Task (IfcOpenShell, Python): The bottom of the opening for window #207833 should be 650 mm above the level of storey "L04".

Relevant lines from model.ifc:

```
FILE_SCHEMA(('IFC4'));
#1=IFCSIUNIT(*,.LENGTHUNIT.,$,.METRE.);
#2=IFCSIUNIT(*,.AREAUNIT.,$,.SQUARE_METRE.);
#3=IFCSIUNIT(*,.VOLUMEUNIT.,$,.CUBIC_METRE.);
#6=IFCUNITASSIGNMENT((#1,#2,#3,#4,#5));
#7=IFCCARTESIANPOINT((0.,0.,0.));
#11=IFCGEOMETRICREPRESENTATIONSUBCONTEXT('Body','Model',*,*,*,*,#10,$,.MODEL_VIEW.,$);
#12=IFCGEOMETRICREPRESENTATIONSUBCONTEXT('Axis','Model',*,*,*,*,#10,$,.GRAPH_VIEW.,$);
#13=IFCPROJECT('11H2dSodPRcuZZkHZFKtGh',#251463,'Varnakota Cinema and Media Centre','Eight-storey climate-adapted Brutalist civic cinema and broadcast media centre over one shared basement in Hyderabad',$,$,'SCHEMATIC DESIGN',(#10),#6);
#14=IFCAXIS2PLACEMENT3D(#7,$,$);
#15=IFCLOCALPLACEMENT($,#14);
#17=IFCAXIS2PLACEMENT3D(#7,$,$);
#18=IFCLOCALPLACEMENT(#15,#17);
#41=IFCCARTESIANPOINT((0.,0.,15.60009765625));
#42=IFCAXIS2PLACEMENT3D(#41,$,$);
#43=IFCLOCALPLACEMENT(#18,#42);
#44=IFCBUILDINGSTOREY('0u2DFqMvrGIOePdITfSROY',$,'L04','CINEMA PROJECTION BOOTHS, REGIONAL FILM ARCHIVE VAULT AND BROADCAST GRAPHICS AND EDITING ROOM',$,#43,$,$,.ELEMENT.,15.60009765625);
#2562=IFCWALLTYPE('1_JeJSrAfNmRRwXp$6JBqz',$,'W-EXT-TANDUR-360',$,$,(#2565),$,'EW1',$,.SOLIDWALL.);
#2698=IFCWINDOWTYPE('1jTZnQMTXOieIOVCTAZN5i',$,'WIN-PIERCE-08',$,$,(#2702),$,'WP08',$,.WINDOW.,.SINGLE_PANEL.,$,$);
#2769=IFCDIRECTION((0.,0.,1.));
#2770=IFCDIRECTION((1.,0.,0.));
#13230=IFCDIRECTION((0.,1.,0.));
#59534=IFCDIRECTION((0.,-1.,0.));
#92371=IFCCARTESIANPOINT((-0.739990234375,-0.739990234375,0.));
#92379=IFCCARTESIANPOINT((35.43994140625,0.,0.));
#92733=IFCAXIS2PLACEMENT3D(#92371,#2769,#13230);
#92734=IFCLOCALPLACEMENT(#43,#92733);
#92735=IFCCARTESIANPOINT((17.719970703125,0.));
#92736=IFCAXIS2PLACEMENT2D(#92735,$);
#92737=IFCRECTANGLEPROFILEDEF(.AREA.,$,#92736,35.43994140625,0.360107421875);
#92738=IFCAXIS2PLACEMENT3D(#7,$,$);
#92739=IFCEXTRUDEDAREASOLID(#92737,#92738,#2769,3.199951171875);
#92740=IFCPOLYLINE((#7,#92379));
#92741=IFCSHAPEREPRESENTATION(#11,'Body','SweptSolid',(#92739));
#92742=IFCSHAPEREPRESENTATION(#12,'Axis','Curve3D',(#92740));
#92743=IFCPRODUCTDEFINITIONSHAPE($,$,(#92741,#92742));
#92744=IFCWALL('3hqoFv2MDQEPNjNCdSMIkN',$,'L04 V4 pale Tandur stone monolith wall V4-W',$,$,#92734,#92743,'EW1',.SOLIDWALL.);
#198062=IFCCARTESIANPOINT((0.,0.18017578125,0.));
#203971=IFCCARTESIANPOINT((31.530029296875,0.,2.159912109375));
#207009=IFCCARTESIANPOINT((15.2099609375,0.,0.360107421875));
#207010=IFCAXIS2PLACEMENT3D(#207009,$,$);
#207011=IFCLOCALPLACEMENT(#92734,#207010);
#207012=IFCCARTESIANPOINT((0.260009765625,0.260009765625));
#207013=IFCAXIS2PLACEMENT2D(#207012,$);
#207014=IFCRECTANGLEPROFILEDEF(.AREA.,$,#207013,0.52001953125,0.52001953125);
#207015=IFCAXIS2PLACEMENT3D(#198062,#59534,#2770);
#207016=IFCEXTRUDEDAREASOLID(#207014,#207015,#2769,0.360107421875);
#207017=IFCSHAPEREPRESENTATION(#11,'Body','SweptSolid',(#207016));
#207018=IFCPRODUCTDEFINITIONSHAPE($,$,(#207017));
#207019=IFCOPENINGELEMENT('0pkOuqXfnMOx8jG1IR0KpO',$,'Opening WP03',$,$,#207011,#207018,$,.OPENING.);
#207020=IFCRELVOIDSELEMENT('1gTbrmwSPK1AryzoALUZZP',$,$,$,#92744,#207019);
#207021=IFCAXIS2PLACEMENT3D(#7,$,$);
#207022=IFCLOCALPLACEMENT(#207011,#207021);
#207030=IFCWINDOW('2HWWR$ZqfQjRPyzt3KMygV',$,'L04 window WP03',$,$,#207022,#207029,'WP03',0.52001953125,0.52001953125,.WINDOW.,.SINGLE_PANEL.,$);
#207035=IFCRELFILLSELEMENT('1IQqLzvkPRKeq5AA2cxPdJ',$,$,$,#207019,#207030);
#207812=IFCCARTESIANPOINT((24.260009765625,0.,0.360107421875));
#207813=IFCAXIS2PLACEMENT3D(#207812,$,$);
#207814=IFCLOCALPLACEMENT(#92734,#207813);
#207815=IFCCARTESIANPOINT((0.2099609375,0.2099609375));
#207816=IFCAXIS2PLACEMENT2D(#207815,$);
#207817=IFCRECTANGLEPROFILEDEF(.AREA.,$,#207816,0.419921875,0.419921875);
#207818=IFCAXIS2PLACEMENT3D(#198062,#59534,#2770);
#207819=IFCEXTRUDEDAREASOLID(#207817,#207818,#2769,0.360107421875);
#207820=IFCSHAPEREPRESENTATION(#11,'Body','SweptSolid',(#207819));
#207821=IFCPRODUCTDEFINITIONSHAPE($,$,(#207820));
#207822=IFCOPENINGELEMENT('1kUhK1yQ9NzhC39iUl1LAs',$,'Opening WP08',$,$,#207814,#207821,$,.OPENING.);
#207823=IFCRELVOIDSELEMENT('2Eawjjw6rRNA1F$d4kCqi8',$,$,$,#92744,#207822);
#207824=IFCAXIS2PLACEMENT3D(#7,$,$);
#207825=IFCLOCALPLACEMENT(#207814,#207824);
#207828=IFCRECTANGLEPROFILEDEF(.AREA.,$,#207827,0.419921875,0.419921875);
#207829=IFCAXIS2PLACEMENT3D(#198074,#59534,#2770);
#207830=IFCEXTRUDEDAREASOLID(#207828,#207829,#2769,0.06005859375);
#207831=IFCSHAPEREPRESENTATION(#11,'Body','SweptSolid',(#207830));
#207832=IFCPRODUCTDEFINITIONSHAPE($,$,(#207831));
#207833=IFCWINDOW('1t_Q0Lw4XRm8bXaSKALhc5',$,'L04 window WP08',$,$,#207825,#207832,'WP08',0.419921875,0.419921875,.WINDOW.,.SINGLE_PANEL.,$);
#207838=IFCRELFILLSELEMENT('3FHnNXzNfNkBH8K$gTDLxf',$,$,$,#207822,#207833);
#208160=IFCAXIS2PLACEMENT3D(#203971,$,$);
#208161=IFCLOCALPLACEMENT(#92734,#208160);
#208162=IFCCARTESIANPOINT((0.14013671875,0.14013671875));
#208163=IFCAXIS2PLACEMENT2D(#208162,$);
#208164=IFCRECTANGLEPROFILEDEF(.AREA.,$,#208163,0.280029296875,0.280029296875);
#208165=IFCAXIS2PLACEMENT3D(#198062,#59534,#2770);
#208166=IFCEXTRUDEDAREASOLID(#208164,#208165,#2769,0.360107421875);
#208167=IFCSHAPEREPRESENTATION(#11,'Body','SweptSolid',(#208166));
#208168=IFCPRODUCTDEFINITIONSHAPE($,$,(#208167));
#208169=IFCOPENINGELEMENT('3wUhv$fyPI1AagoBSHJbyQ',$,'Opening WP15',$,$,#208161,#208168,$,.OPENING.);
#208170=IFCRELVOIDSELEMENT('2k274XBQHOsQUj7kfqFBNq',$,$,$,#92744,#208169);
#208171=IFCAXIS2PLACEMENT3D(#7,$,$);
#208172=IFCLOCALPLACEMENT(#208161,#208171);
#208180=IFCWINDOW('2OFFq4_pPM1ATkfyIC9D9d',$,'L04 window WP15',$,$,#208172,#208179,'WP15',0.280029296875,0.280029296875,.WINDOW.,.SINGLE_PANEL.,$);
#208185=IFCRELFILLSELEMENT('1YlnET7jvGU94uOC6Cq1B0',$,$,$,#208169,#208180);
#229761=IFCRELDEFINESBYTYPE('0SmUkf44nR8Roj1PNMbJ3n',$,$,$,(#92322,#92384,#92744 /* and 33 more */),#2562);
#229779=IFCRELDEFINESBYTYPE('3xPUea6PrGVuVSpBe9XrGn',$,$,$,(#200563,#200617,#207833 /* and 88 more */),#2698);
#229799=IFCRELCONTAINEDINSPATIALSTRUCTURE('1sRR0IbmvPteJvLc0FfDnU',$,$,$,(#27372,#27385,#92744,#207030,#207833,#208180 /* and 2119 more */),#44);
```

```python
import numpy as np
import ifcopenshell
import ifcopenshell.api.geometry
import ifcopenshell.geom
import ifcopenshell.util.element
import ifcopenshell.util.placement
import ifcopenshell.util.shape
import ifcopenshell.util.unit

model = ifcopenshell.open("model.ifc")
unit_scale = ifcopenshell.util.unit.calculate_unit_scale(model)

window = model.by_guid("1t_Q0Lw4XRm8bXaSKALhc5")
opening = window.FillsVoids[0].RelatingOpeningElement
storey = ifcopenshell.util.element.get_container(window, ifc_class="IfcBuildingStorey")
level = ifcopenshell.util.placement.get_local_placement(storey.ObjectPlacement)[2, 3]

# The opening's origin need not be at the sill, so measure its lowest point.
shape = ifcopenshell.geom.create_shape(ifcopenshell.geom.settings(), opening)
bottom = ifcopenshell.util.shape.get_shape_bottom_elevation(shape, shape.geometry) / unit_scale
dz = level + 0.65 / unit_scale - bottom

shift = np.array([0.0, 0.0, dz])
# The window is placed relative to its opening, so it follows when the opening moves.
matrix = ifcopenshell.util.placement.get_local_placement(opening.ObjectPlacement)
matrix[:3, 3] += shift
ifcopenshell.api.geometry.edit_object_placement(
    model, product=opening, matrix=matrix, is_si=False, should_transform_children=True
)

print(f"moved by {dz * unit_scale:+.3f} m")

model.write("model_updated.ifc")
```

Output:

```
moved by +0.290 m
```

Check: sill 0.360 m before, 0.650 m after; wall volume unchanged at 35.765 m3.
